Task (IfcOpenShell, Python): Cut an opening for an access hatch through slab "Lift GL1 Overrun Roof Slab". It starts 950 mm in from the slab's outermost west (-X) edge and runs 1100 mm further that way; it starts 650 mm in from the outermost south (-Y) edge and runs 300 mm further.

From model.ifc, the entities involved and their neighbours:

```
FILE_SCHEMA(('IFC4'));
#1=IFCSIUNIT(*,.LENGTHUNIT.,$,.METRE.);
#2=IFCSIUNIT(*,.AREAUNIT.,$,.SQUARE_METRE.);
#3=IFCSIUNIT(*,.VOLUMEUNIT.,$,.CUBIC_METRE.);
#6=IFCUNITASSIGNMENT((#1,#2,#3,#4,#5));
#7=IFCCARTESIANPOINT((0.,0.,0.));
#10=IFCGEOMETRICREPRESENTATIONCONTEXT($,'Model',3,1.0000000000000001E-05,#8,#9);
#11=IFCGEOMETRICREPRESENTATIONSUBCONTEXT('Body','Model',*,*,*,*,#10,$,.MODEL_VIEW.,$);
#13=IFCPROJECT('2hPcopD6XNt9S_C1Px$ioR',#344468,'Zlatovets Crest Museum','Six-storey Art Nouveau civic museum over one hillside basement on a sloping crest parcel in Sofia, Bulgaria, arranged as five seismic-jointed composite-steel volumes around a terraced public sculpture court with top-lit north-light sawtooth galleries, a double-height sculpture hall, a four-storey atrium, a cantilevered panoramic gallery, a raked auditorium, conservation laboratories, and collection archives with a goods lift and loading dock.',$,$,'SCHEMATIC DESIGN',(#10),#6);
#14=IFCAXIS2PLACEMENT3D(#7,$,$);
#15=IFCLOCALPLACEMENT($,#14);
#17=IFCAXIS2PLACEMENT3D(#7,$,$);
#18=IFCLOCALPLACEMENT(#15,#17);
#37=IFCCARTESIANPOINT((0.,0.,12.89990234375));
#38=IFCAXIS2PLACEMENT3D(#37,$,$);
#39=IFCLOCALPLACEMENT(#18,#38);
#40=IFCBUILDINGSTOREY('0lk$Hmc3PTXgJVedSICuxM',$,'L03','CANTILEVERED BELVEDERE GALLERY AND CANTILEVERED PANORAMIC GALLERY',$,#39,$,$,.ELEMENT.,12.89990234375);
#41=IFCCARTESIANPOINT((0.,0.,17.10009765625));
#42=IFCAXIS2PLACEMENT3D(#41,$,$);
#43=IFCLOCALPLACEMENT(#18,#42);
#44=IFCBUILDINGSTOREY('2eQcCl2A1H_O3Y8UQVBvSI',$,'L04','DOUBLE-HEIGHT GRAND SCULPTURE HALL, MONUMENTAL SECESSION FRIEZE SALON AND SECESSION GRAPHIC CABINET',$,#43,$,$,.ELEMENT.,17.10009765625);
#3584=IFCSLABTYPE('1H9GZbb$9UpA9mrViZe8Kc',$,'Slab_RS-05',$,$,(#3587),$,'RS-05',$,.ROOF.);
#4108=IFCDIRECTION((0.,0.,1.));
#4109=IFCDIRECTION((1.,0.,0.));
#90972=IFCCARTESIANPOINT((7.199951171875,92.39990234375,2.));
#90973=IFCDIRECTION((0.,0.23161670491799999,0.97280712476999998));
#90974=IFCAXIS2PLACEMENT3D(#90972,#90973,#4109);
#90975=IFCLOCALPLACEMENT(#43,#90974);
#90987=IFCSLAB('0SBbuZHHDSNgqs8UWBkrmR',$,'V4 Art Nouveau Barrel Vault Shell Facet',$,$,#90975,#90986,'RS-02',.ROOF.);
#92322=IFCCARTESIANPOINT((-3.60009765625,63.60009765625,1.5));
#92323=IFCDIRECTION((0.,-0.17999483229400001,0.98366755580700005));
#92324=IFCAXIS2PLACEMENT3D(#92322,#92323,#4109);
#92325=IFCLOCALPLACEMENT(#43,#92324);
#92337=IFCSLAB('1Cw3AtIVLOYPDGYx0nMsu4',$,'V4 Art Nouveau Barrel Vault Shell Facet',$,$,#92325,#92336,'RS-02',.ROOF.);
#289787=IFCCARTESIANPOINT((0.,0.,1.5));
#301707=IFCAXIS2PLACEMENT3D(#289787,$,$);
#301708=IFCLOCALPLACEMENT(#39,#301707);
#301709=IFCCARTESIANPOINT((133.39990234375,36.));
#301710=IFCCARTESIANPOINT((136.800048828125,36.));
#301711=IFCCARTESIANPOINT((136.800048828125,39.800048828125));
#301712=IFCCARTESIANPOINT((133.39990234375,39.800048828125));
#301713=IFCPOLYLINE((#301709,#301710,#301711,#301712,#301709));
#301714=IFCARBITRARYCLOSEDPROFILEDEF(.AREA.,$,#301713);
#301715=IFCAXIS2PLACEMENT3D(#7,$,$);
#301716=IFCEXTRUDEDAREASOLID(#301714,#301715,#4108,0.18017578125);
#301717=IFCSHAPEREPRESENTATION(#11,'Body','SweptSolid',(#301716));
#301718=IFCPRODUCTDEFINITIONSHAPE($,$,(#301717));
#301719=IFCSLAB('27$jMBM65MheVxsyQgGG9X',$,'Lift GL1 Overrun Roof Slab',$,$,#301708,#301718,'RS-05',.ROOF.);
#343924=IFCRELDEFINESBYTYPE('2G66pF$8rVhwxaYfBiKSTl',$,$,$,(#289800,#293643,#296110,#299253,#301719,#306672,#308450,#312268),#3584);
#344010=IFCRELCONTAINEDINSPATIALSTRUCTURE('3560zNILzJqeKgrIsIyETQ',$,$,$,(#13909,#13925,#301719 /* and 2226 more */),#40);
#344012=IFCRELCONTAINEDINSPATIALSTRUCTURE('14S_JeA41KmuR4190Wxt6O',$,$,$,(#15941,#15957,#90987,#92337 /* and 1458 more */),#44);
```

```python
import numpy as np
import ifcopenshell
import ifcopenshell.api.feature
import ifcopenshell.api.geometry
import ifcopenshell.api.root
import ifcopenshell.geom
import ifcopenshell.util.placement
import ifcopenshell.util.representation
import ifcopenshell.util.shape
import ifcopenshell.util.unit

model = ifcopenshell.open("model.ifc")
unit_scale = ifcopenshell.util.unit.calculate_unit_scale(model)
settings = ifcopenshell.geom.settings()


def volume(element):
    """Net volume in cubic metres, openings subtracted."""
    shape = ifcopenshell.geom.create_shape(settings, element)
    return ifcopenshell.util.shape.get_volume(shape.geometry)


slab = model.by_guid("27$jMBM65MheVxsyQgGG9X")
before = volume(slab)

# Extent in the slab's own axes, in metres. The edges named are its -X and -Y sides.
slab_shape = ifcopenshell.geom.create_shape(settings, slab)
vertices = ifcopenshell.util.shape.get_vertices(slab_shape.geometry)
x_min, y_min, bottom = vertices.min(axis=0)
top = vertices[:, 2].max()

opening = ifcopenshell.api.root.create_entity(model, ifc_class="IfcOpeningElement", name="Access hatch opening", predefined_type="OPENING")
context = ifcopenshell.util.representation.get_context(model, "Model", "Body", "MODEL_VIEW")
width, depth = 1.1, 0.3
outline = [(0.0, 0.0), (width, 0.0), (width, depth), (0.0, depth), (0.0, 0.0)]
# Overshoot both faces by 50 mm so the cut is clean.
shape = ifcopenshell.api.geometry.add_slab_representation(
    model, context=context, depth=top - bottom + 0.1, polyline=outline
)
ifcopenshell.api.geometry.assign_representation(model, product=opening, representation=shape)

matrix = ifcopenshell.util.placement.get_local_placement(slab.ObjectPlacement)
matrix[:, 3] = matrix @ np.append(np.array([x_min + 0.95, y_min + 0.65, bottom - 0.05]) / unit_scale, 1.0)
ifcopenshell.api.geometry.edit_object_placement(model, product=opening, matrix=matrix, is_si=False)
ifcopenshell.api.feature.add_feature(model, feature=opening, element=slab)

after = volume(slab)

print(f"slab volume {before:.3f} -> {after:.3f} m3")

model.write("model_updated.ifc")
```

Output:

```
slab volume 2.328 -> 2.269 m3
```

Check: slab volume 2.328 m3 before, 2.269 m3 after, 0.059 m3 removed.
